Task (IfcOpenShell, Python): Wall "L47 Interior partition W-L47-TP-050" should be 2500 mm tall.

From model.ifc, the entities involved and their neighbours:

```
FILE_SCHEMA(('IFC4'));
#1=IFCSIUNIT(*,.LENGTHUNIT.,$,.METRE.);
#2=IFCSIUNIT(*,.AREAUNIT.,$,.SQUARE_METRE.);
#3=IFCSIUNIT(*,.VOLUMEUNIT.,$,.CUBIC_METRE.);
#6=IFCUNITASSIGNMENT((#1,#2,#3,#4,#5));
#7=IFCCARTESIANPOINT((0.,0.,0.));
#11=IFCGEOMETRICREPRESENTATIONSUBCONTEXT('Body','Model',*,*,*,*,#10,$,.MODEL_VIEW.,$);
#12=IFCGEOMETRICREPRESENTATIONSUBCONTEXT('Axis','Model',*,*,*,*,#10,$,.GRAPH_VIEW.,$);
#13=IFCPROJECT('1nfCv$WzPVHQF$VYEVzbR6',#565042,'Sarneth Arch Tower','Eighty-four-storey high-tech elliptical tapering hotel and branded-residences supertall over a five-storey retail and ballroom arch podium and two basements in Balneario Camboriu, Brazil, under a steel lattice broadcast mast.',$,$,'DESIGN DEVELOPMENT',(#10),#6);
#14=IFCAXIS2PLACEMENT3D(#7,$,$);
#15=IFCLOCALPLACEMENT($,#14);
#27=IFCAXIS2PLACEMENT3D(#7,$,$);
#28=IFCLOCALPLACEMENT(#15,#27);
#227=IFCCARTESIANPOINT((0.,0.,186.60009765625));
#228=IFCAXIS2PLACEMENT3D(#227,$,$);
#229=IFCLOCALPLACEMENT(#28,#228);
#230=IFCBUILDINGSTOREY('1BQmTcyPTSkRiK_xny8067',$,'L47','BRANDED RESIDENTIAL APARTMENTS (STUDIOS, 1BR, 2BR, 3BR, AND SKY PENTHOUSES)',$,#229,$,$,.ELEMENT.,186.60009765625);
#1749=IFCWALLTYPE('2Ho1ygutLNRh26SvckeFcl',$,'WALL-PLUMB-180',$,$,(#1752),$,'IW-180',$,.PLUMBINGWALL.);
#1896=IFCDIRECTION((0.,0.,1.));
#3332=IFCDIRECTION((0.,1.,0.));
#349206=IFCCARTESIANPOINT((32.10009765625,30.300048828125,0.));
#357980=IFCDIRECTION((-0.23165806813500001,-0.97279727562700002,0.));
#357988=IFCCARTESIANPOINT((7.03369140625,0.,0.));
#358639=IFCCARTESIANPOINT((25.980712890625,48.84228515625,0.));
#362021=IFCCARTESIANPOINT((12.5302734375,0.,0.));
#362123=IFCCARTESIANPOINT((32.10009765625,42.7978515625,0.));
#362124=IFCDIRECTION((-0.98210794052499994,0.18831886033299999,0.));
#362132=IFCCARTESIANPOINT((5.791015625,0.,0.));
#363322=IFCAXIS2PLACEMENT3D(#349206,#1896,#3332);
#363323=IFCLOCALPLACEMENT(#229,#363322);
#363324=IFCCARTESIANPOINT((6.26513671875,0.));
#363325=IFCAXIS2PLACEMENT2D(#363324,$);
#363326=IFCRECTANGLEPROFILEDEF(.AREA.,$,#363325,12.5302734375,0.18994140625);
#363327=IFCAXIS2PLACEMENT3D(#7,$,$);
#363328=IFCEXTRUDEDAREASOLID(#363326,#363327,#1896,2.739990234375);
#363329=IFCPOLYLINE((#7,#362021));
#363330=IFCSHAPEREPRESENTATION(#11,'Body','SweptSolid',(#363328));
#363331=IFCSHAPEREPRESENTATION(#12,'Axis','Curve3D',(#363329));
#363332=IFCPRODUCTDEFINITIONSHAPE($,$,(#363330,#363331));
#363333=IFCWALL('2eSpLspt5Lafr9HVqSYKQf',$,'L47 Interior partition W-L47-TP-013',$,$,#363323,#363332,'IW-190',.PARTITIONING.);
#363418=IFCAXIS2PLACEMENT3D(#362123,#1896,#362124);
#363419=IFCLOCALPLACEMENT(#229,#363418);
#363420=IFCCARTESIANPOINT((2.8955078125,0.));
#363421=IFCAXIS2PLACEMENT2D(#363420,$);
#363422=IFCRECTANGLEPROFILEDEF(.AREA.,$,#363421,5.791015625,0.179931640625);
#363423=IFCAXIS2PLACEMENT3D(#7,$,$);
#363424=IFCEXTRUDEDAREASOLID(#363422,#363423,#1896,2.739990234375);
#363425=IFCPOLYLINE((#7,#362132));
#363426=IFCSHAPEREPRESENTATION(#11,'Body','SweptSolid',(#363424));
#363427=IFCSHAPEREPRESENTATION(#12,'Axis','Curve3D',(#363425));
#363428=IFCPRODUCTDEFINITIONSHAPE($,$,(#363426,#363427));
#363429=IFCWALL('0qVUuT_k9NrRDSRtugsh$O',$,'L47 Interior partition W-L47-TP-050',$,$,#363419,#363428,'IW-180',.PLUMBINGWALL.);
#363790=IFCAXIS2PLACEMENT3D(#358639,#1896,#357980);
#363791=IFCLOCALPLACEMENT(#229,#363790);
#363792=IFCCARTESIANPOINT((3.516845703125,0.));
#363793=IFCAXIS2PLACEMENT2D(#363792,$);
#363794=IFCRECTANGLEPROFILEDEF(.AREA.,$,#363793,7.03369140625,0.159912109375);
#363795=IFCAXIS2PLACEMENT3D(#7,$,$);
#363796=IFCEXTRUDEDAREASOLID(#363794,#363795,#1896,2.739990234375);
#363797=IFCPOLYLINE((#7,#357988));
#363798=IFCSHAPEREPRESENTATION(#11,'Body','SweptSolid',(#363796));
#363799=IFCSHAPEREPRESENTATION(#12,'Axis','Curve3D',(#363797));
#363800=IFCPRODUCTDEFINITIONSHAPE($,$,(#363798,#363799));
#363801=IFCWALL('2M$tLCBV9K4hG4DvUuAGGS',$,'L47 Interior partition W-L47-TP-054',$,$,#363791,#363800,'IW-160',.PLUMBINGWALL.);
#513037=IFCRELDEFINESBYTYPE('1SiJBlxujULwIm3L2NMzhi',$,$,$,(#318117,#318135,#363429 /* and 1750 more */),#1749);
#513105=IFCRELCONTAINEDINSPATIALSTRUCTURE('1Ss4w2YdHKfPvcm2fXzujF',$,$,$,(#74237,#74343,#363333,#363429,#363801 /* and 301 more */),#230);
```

```python
import ifcopenshell
import ifcopenshell.geom
import ifcopenshell.util.representation
import ifcopenshell.util.shape
import ifcopenshell.util.unit

model = ifcopenshell.open("model.ifc")
unit_scale = ifcopenshell.util.unit.calculate_unit_scale(model)
settings = ifcopenshell.geom.settings()


def volume(element):
    """Net volume in cubic metres, openings subtracted."""
    shape = ifcopenshell.geom.create_shape(settings, element)
    return ifcopenshell.util.shape.get_volume(shape.geometry)


wall = model.by_id(363429)
before = volume(wall)

body = ifcopenshell.util.representation.get_representation(wall, "Model", "Body")
solid = body.Items[0]
old_height = solid.Depth
solid.Depth = 2.5 / unit_scale
after = volume(wall)

print(f"height {old_height:g} -> {solid.Depth:g}, volume {before:.3f} -> {after:.3f} m3")

model.write("model_v2.ifc")
```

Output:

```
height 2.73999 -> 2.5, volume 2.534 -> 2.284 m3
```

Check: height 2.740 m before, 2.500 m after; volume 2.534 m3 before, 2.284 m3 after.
